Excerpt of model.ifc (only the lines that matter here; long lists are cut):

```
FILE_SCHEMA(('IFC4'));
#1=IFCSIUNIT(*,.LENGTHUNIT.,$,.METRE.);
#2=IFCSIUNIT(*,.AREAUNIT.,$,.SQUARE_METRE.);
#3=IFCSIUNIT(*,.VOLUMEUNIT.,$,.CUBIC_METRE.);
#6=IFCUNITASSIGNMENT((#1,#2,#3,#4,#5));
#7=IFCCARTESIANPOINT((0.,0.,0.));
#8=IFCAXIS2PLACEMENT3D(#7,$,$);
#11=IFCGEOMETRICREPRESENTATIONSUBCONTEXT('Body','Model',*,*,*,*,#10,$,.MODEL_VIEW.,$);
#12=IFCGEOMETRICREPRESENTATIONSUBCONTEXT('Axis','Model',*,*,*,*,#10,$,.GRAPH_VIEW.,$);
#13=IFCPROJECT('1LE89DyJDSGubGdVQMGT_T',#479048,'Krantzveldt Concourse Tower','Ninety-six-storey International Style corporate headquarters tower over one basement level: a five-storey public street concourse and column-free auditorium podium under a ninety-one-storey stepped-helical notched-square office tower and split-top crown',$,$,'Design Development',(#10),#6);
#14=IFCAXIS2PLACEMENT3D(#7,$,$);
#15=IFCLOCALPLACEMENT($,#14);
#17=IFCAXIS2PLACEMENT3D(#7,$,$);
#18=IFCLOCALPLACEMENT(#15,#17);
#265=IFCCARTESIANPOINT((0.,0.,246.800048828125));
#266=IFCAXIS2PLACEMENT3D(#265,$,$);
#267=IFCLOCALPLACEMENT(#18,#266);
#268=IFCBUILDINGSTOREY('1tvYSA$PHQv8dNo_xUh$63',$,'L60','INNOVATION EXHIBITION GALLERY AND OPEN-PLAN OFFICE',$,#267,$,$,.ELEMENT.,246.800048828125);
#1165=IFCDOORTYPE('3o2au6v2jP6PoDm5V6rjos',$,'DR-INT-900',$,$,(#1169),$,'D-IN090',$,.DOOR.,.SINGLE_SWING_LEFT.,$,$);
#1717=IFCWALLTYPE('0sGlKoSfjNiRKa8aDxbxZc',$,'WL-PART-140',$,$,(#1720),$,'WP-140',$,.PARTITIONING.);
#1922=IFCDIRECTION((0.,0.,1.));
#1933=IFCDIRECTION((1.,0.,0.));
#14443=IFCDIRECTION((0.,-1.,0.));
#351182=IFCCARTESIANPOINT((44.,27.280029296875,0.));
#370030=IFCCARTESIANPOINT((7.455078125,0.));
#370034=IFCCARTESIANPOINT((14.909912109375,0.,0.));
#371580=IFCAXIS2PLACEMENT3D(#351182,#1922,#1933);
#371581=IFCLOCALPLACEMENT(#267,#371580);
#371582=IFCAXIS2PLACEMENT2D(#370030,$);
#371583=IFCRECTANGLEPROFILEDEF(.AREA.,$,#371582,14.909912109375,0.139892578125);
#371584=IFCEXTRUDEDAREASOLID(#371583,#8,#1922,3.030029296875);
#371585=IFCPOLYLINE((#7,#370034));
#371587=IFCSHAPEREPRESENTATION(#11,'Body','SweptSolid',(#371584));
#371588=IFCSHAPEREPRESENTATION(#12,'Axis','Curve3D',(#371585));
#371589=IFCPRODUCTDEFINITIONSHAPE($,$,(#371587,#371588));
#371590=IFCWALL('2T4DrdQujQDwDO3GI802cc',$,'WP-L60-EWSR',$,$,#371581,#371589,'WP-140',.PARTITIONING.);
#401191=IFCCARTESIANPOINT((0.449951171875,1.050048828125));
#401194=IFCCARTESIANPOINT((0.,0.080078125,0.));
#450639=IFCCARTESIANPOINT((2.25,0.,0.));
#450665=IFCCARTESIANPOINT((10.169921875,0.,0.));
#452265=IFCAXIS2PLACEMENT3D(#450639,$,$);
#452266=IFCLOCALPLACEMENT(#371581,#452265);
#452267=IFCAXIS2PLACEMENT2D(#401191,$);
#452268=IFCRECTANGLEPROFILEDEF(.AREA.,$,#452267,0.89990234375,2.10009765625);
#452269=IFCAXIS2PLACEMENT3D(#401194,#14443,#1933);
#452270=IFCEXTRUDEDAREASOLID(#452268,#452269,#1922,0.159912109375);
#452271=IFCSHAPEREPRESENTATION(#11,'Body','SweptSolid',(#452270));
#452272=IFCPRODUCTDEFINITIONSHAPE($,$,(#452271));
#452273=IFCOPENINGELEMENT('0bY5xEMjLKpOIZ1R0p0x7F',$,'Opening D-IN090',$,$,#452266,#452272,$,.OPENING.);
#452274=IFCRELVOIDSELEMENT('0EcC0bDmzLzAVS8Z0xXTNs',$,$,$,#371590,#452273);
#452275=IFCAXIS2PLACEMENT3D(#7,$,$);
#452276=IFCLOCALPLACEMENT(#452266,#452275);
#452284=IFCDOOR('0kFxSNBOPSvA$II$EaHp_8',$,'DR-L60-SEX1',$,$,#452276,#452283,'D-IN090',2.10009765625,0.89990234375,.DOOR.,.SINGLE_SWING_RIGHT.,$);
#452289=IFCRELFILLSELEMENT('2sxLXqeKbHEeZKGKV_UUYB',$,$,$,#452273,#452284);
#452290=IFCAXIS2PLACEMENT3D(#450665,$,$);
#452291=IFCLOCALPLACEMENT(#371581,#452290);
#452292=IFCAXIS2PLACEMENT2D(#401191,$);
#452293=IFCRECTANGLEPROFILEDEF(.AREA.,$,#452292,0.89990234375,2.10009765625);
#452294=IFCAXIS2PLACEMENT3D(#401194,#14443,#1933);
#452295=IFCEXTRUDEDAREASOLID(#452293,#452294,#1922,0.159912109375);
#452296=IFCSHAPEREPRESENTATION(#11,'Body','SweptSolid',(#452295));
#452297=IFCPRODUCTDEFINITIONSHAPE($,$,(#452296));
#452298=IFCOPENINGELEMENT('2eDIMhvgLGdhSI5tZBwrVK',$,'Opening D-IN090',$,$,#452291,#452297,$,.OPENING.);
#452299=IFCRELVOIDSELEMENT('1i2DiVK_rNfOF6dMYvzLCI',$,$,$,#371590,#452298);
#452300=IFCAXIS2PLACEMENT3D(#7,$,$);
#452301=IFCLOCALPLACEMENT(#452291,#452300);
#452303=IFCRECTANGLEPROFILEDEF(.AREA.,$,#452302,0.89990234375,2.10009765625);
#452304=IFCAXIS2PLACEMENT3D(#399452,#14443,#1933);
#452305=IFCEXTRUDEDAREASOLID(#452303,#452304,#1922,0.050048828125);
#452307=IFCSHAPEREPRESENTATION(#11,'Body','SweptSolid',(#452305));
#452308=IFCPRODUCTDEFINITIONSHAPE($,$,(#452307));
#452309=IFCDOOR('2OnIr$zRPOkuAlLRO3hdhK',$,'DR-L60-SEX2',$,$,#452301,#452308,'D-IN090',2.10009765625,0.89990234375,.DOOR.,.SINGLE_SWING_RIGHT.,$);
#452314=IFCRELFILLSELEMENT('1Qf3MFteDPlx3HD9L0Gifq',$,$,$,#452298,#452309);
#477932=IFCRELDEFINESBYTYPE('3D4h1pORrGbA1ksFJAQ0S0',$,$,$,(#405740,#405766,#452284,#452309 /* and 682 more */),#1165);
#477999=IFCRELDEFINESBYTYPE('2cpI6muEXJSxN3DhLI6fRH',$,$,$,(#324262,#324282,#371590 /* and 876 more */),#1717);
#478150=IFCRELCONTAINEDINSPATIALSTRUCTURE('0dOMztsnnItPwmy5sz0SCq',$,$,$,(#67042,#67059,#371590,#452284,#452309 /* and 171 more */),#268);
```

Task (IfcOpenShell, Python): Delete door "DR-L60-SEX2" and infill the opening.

```python
import ifcopenshell
import ifcopenshell.api.feature
import ifcopenshell.api.root
import ifcopenshell.geom
import ifcopenshell.util.shape

model = ifcopenshell.open("model.ifc")
settings = ifcopenshell.geom.settings()


def volume(element):
    """Net volume in cubic metres, openings subtracted."""
    shape = ifcopenshell.geom.create_shape(settings, element)
    return ifcopenshell.util.shape.get_volume(shape.geometry)


door = model.by_guid("2OnIr$zRPOkuAlLRO3hdhK")
opening = door.FillsVoids[0].RelatingOpeningElement
wall = opening.VoidsElements[0].RelatingBuildingElement
before = volume(wall)

ifcopenshell.api.root.remove_product(model, product=door)
ifcopenshell.api.feature.remove_feature(model, feature=opening)

after = volume(wall)

print(f"wall volume {before:.3f} -> {after:.3f} m3")

model.write("model_updated.ifc")
```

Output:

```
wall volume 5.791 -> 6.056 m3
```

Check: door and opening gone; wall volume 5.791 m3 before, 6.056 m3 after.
